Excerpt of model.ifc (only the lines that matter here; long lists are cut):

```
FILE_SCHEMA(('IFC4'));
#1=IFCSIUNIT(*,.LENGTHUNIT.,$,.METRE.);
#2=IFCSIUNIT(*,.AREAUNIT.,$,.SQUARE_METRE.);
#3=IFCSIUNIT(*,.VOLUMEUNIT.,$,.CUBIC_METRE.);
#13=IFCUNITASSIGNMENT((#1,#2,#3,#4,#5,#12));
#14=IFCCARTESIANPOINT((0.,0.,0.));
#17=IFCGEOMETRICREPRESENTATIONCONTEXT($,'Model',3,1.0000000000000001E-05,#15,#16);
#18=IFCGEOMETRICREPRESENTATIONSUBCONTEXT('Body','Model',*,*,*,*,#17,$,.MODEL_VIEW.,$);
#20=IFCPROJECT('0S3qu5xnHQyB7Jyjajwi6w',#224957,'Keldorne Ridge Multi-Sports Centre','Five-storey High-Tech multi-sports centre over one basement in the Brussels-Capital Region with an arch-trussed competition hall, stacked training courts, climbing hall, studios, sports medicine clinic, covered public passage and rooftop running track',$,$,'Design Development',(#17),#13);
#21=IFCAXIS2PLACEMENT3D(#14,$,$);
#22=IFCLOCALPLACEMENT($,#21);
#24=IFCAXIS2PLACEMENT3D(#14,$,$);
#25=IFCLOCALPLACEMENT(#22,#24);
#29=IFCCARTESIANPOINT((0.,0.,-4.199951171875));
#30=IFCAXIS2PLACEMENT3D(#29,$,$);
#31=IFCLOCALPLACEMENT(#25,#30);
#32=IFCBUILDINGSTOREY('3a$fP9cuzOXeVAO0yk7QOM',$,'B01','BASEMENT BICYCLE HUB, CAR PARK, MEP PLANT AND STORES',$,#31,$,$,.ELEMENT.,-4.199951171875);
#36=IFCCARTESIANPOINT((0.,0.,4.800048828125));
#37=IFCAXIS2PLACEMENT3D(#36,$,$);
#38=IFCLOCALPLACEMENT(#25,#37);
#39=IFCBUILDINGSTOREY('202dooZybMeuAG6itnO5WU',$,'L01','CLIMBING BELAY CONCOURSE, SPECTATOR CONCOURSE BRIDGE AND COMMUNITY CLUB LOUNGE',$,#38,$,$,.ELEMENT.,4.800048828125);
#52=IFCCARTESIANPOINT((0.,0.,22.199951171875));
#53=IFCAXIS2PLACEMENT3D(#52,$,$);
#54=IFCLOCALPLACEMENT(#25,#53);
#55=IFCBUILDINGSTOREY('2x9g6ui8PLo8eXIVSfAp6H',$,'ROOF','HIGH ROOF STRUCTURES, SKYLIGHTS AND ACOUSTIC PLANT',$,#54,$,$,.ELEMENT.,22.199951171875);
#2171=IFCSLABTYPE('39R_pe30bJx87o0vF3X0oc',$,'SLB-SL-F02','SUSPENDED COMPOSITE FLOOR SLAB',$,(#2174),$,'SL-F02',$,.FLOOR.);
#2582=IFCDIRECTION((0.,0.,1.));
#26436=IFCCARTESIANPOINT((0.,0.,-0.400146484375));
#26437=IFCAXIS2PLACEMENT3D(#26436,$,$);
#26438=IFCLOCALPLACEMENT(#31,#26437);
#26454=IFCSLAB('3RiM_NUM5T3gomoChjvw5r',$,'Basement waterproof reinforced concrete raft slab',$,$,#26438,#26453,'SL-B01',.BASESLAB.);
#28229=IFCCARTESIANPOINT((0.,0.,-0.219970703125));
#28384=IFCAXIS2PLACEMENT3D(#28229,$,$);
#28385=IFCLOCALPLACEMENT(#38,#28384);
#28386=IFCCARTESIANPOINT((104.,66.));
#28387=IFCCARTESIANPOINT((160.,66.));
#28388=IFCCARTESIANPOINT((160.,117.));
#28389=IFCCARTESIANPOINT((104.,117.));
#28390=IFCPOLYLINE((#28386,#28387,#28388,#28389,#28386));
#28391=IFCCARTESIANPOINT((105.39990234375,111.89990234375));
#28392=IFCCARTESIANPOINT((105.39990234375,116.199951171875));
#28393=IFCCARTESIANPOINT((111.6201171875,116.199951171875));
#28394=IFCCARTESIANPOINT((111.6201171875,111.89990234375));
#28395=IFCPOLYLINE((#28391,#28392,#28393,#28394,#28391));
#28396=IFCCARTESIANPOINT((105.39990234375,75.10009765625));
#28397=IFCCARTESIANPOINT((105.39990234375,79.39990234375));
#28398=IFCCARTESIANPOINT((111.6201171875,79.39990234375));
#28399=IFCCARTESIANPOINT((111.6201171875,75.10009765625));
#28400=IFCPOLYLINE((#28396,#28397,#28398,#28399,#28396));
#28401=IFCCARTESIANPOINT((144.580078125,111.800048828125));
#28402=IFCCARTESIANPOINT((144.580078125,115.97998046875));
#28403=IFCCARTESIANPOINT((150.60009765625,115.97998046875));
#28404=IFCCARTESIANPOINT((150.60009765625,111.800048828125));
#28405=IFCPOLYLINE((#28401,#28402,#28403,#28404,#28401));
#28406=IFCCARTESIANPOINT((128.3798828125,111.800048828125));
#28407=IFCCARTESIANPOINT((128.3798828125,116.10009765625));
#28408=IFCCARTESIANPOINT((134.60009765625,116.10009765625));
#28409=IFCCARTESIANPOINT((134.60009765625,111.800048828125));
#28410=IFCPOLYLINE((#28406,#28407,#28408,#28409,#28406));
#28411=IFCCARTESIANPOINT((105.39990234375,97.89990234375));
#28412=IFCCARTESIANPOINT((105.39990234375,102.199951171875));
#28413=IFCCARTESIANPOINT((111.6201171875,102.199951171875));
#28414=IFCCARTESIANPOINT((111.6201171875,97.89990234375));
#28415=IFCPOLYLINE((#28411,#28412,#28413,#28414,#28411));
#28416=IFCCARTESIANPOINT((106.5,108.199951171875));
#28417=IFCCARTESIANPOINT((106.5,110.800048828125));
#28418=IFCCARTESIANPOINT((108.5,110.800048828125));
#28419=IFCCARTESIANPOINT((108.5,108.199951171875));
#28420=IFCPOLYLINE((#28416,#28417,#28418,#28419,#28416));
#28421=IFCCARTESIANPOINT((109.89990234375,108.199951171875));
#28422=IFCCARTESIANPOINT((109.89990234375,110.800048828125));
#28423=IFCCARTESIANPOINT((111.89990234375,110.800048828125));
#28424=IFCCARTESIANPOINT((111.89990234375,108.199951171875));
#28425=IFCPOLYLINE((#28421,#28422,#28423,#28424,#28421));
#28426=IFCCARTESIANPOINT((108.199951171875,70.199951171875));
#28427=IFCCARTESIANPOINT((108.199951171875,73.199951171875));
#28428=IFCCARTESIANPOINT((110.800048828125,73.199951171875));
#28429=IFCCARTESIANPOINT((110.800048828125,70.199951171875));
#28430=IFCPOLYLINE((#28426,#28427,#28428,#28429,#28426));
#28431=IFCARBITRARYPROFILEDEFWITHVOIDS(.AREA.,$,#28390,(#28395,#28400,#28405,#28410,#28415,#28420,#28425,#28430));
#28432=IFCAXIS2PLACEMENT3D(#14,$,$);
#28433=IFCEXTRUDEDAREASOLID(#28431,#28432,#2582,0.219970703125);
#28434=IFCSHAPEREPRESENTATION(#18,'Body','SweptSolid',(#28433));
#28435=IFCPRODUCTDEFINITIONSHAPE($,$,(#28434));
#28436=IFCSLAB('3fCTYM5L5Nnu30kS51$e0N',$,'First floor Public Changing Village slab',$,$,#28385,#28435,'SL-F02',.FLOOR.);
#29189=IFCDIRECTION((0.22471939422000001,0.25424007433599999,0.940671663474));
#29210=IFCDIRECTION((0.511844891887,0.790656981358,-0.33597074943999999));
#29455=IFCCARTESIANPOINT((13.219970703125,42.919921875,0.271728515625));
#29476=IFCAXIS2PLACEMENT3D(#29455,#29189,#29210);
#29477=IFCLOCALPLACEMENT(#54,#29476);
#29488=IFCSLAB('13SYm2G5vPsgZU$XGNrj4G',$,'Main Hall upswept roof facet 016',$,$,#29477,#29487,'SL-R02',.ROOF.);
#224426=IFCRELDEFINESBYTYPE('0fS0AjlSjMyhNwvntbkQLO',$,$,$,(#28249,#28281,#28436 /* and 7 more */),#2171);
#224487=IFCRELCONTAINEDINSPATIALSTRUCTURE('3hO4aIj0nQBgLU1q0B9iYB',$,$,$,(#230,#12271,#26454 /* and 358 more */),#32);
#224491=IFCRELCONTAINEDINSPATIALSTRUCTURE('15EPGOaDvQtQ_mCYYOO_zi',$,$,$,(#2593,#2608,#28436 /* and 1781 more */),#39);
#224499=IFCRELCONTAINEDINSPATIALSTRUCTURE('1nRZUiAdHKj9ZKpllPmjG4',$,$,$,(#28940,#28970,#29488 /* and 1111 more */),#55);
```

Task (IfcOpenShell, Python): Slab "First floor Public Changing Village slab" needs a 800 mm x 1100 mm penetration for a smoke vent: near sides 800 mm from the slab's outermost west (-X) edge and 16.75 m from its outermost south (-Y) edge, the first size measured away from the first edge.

```python
import numpy as np
import ifcopenshell
import ifcopenshell.api.feature
import ifcopenshell.api.geometry
import ifcopenshell.api.root
import ifcopenshell.geom
import ifcopenshell.util.placement
import ifcopenshell.util.representation
import ifcopenshell.util.shape
import ifcopenshell.util.unit

model = ifcopenshell.open("model.ifc")
unit_scale = ifcopenshell.util.unit.calculate_unit_scale(model)
settings = ifcopenshell.geom.settings()


def volume(element):
    """Net volume in cubic metres, openings subtracted."""
    shape = ifcopenshell.geom.create_shape(settings, element)
    return ifcopenshell.util.shape.get_volume(shape.geometry)


slab = model.by_id(28436)
before = volume(slab)

# Extent in the slab's own axes, in metres. The edges named are its -X and -Y sides.
slab_shape = ifcopenshell.geom.create_shape(settings, slab)
vertices = ifcopenshell.util.shape.get_vertices(slab_shape.geometry)
x_min, y_min, bottom = vertices.min(axis=0)
top = vertices[:, 2].max()

opening = ifcopenshell.api.root.create_entity(model, ifc_class="IfcOpeningElement", name="Smoke vent opening", predefined_type="OPENING")
context = ifcopenshell.util.representation.get_context(model, "Model", "Body", "MODEL_VIEW")
width, depth = 0.8, 1.1
outline = [(0.0, 0.0), (width, 0.0), (width, depth), (0.0, depth), (0.0, 0.0)]
# Overshoot both faces by 50 mm so the cut is clean.
shape = ifcopenshell.api.geometry.add_slab_representation(
    model, context=context, depth=top - bottom + 0.1, polyline=outline
)
ifcopenshell.api.geometry.assign_representation(model, product=opening, representation=shape)

matrix = ifcopenshell.util.placement.get_local_placement(slab.ObjectPlacement)
matrix[:, 3] = matrix @ np.append(np.array([x_min + 0.8, y_min + 16.75, bottom - 0.05]) / unit_scale, 1.0)
ifcopenshell.api.geometry.edit_object_placement(model, product=opening, matrix=matrix, is_si=False)
ifcopenshell.api.feature.add_feature(model, feature=opening, element=slab)

after = volume(slab)

print(f"slab volume {before:.3f} -> {after:.3f} m3")

model.write("model_updated.ifc")
```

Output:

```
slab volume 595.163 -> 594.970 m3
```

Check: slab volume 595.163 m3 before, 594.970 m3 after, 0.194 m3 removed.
